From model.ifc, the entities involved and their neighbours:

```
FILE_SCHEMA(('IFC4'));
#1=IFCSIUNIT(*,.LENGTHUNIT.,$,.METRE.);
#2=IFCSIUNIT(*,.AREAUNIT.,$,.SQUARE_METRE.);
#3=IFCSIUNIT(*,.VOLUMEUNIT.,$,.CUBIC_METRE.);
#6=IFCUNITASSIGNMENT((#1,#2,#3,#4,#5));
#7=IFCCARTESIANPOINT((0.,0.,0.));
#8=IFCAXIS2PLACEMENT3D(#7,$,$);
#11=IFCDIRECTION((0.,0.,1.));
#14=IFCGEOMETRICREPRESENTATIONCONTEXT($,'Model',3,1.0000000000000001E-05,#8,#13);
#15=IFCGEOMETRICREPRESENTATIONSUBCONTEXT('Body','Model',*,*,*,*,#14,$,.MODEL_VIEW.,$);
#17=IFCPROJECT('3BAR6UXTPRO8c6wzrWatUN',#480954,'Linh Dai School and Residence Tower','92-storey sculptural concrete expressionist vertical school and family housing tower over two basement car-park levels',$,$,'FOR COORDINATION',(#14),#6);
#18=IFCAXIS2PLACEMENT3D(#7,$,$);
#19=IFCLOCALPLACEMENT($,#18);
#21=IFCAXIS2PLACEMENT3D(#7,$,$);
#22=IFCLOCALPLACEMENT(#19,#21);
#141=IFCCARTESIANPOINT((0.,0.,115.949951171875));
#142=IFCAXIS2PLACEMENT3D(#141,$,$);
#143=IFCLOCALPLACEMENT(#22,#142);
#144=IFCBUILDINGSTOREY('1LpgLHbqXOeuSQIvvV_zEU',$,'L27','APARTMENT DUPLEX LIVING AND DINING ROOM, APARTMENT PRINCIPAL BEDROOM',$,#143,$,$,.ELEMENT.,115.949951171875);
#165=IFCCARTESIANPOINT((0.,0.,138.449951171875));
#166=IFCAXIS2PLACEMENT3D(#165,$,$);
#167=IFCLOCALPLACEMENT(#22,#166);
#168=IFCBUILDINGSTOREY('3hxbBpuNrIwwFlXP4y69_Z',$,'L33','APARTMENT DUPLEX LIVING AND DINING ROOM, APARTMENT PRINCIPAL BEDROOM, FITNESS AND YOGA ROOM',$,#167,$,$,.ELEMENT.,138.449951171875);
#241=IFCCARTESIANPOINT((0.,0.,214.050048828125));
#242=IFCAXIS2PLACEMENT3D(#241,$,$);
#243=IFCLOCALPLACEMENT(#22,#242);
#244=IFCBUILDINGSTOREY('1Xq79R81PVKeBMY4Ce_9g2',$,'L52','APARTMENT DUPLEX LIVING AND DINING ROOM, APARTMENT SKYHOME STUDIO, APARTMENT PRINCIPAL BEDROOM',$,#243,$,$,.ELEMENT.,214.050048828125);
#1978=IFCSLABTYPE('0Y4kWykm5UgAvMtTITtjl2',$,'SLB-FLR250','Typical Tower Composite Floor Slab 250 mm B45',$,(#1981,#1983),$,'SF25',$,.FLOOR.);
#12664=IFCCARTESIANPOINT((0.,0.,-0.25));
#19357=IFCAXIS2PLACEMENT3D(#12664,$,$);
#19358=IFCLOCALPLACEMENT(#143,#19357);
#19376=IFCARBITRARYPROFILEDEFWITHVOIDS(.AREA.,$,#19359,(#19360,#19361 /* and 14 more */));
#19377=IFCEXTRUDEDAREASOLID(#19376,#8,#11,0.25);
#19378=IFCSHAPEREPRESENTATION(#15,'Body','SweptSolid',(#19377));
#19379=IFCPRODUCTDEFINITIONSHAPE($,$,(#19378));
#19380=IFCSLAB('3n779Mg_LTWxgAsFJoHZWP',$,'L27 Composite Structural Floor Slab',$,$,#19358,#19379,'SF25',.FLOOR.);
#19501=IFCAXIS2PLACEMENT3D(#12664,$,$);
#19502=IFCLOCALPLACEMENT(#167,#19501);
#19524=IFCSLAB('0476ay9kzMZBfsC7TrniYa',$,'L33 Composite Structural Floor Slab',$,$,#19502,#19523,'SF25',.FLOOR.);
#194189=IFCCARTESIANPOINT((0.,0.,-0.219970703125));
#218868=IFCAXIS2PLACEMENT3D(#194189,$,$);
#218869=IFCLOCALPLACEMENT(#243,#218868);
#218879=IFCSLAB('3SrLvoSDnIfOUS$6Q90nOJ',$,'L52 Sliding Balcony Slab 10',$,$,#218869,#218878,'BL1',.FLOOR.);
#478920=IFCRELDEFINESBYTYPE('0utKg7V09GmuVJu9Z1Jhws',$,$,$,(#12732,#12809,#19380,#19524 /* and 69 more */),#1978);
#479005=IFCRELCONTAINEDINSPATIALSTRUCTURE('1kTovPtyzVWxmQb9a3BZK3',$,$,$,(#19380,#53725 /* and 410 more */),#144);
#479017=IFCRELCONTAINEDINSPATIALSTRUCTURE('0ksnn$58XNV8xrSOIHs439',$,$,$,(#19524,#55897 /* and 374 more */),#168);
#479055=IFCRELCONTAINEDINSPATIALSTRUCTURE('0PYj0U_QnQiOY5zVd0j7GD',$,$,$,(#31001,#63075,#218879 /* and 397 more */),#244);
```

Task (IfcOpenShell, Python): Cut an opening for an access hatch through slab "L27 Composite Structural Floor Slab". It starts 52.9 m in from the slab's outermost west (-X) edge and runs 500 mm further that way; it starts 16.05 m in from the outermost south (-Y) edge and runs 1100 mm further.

```python
import numpy as np
import ifcopenshell
import ifcopenshell.api.feature
import ifcopenshell.api.geometry
import ifcopenshell.api.root
import ifcopenshell.geom
import ifcopenshell.util.placement
import ifcopenshell.util.representation
import ifcopenshell.util.shape
import ifcopenshell.util.unit

model = ifcopenshell.open("model.ifc")
unit_scale = ifcopenshell.util.unit.calculate_unit_scale(model)
settings = ifcopenshell.geom.settings()


def volume(element):
    """Net volume in cubic metres, openings subtracted."""
    shape = ifcopenshell.geom.create_shape(settings, element)
    return ifcopenshell.util.shape.get_volume(shape.geometry)


slab = model.by_guid("3n779Mg_LTWxgAsFJoHZWP")
before = volume(slab)

# Extent in the slab's own axes, in metres. The edges named are its -X and -Y sides.
slab_shape = ifcopenshell.geom.create_shape(settings, slab)
vertices = ifcopenshell.util.shape.get_vertices(slab_shape.geometry)
x_min, y_min, bottom = vertices.min(axis=0)
top = vertices[:, 2].max()

opening = ifcopenshell.api.root.create_entity(model, ifc_class="IfcOpeningElement", name="Access hatch opening", predefined_type="OPENING")
context = ifcopenshell.util.representation.get_context(model, "Model", "Body", "MODEL_VIEW")
width, depth = 0.5, 1.1
outline = [(0.0, 0.0), (width, 0.0), (width, depth), (0.0, depth), (0.0, 0.0)]
# Overshoot both faces by 50 mm so the cut is clean.
shape = ifcopenshell.api.geometry.add_slab_representation(
    model, context=context, depth=top - bottom + 0.1, polyline=outline
)
ifcopenshell.api.geometry.assign_representation(model, product=opening, representation=shape)

matrix = ifcopenshell.util.placement.get_local_placement(slab.ObjectPlacement)
matrix[:, 3] = matrix @ np.append(np.array([x_min + 52.9, y_min + 16.05, bottom - 0.05]) / unit_scale, 1.0)
ifcopenshell.api.geometry.edit_object_placement(model, product=opening, matrix=matrix, is_si=False)
ifcopenshell.api.feature.add_feature(model, feature=opening, element=slab)

after = volume(slab)

print(f"slab volume {before:.3f} -> {after:.3f} m3")

model.write("model-out.ifc")
```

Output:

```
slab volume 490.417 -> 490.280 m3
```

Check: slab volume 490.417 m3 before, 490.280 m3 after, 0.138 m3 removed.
